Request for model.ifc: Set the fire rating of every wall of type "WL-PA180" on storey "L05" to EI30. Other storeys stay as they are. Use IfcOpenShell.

First a look at what the model holds.

```python
import ifcopenshell
import ifcopenshell.util.element

model = ifcopenshell.open("model.ifc")
print(model.schema)
storey = next(s for s in model.by_type("IfcBuildingStorey") if s.Name == "L05")
walls = [e for e in ifcopenshell.util.element.get_decomposition(storey) if e.is_a("IfcWall")]
seen = {}
for e in walls:
    element_type = ifcopenshell.util.element.get_type(e)
    key = (element_type.Name if element_type != e and element_type else None, ifcopenshell.util.element.get_pset(e, "Pset_WallCommon", "FireRating"))
    seen[key] = seen.get(key, 0) + 1
for (name, value), count in sorted(seen.items(), key=str):
    print(count, "x", name, "|", value)
```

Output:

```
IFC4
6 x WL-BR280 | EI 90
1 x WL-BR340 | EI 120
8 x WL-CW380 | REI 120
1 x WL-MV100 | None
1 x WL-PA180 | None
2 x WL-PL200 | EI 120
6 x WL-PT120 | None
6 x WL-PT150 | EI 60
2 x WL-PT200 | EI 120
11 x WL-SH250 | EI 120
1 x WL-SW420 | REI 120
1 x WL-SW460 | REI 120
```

```python
import ifcopenshell
import ifcopenshell.api.pset
import ifcopenshell.util.element

model = ifcopenshell.open("model.ifc")

storey = next(s for s in model.by_type("IfcBuildingStorey") if s.Name == "L05")
walls = [e for e in ifcopenshell.util.element.get_decomposition(storey) if e.is_a("IfcWall")]

count = 0
for e in walls:
    element_type = ifcopenshell.util.element.get_type(e)
    if element_type in (None, e) or element_type.Name != "WL-PA180":
        continue
    # add_pset returns the element's existing set when there is one.
    pset = ifcopenshell.api.pset.add_pset(model, product=e, name="Pset_WallCommon")
    ifcopenshell.api.pset.edit_pset(model, pset=pset, properties={"FireRating": "EI30"})
    count += 1

print(count, "walls updated")

model.write("model-out.ifc")
```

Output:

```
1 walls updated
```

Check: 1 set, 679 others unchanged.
